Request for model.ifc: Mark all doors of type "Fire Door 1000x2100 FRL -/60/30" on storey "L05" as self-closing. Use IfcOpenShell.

First a look at what the model holds.

```python
import ifcopenshell
import ifcopenshell.util.element

model = ifcopenshell.open("model.ifc")
print(model.schema)
storey = next(s for s in model.by_type("IfcBuildingStorey") if s.Name == "L05")
doors = [e for e in ifcopenshell.util.element.get_decomposition(storey) if e.is_a("IfcDoor")]
seen = {}
for e in doors:
    element_type = ifcopenshell.util.element.get_type(e)
    key = (element_type.Name if element_type != e and element_type else None, ifcopenshell.util.element.get_pset(e, "Pset_DoorCommon", "SelfClosing"))
    seen[key] = seen.get(key, 0) + 1
for (name, value), count in sorted(seen.items(), key=str):
    print(count, "x", name, "|", value)
```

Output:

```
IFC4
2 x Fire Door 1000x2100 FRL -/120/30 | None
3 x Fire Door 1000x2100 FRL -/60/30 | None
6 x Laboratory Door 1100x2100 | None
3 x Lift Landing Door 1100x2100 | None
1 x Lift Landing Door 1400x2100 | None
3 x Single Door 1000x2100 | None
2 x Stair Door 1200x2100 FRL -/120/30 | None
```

```python
import ifcopenshell
import ifcopenshell.api.pset
import ifcopenshell.util.element

model = ifcopenshell.open("model.ifc")

storey = next(s for s in model.by_type("IfcBuildingStorey") if s.Name == "L05")
doors = [e for e in ifcopenshell.util.element.get_decomposition(storey) if e.is_a("IfcDoor")]

count = 0
for e in doors:
    element_type = ifcopenshell.util.element.get_type(e)
    if element_type in (None, e) or element_type.Name != "Fire Door 1000x2100 FRL -/60/30":
        continue
    # add_pset returns the element's existing set when there is one.
    pset = ifcopenshell.api.pset.add_pset(model, product=e, name="Pset_DoorCommon")
    ifcopenshell.api.pset.edit_pset(model, pset=pset, properties={"SelfClosing": True})
    count += 1

print(count, "doors updated")

model.write("model_v2.ifc")
```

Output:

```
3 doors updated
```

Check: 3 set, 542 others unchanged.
